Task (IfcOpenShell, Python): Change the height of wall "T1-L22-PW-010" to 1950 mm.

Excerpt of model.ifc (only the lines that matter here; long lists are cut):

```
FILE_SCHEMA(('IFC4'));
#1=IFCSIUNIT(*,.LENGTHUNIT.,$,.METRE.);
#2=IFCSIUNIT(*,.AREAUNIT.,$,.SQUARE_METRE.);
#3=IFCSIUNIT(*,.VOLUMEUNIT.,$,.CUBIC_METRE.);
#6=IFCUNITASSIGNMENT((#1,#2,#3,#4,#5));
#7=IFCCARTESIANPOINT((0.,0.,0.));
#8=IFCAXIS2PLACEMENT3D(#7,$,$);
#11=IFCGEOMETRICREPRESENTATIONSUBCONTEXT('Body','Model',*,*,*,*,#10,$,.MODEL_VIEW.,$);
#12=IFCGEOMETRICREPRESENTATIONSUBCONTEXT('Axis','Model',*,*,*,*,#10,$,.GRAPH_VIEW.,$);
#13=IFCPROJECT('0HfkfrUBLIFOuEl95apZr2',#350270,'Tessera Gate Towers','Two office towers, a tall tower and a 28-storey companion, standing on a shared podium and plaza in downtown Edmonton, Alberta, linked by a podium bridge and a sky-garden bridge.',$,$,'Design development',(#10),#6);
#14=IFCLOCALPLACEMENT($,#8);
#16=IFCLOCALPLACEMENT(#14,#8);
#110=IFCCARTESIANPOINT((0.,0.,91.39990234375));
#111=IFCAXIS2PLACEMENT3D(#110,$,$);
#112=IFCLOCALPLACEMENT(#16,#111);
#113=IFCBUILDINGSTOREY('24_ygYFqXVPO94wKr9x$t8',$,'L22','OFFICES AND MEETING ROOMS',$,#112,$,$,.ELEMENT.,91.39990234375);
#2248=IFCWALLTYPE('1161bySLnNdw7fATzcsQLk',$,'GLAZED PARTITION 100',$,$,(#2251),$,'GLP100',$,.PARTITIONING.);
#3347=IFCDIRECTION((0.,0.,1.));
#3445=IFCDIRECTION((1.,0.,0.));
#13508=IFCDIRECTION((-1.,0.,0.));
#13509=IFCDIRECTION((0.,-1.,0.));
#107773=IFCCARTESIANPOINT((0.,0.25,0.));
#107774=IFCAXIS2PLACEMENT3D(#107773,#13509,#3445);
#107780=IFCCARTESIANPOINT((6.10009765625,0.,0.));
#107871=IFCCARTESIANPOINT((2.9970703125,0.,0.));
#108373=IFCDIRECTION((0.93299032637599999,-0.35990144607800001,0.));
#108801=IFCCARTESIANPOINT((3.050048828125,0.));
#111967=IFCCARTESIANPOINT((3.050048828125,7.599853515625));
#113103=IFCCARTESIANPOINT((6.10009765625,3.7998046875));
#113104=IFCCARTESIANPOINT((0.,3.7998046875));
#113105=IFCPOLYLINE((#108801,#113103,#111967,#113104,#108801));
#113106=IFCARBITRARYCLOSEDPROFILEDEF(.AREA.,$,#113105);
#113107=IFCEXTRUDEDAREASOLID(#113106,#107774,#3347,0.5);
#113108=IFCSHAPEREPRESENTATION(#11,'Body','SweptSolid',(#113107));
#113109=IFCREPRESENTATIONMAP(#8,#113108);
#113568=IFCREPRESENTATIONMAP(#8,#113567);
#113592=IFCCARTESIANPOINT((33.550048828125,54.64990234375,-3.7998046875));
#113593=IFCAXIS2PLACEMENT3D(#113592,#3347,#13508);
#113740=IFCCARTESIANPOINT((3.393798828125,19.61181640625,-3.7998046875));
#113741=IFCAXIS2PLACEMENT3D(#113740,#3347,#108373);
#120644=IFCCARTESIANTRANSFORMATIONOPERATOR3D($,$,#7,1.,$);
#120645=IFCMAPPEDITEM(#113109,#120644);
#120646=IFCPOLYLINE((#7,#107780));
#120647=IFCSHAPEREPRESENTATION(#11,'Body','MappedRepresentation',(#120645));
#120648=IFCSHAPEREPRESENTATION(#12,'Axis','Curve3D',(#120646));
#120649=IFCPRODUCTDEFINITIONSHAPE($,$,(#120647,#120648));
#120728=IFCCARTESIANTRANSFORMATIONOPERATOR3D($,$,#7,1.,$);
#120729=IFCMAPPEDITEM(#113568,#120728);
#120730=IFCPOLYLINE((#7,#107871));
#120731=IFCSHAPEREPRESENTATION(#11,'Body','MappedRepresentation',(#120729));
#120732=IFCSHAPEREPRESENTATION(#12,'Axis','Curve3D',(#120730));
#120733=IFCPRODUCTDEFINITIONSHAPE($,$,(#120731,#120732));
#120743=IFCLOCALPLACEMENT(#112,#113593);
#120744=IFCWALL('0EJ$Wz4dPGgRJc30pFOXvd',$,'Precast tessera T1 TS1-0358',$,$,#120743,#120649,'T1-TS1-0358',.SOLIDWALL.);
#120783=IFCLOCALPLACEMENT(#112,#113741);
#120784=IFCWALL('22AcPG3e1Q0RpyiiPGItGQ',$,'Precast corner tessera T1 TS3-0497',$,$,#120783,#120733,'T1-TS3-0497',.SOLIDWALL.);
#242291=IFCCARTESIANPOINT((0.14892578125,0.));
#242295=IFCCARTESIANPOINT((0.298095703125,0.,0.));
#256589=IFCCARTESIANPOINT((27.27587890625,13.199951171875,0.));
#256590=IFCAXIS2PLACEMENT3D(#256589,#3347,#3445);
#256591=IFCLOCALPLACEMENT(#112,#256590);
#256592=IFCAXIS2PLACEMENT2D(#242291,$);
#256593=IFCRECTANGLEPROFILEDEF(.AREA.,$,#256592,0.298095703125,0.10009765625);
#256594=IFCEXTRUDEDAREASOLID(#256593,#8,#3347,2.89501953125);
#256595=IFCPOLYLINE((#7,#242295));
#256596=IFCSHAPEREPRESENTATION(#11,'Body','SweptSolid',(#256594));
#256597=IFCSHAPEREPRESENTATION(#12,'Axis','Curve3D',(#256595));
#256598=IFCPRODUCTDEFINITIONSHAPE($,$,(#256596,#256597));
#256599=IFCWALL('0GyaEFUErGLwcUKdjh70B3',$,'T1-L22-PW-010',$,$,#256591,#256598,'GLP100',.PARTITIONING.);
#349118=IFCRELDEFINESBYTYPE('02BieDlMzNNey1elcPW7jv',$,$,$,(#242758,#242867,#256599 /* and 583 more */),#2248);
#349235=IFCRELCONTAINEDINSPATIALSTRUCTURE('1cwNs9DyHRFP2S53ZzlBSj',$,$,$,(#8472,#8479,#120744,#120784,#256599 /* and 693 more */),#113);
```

```python
import ifcopenshell
import ifcopenshell.geom
import ifcopenshell.util.representation
import ifcopenshell.util.shape

model = ifcopenshell.open("model.ifc")
settings = ifcopenshell.geom.settings()


def volume(element):
    """Net volume in cubic metres, openings subtracted."""
    shape = ifcopenshell.geom.create_shape(settings, element)
    return ifcopenshell.util.shape.get_volume(shape.geometry)


wall = model.by_id(256599)
before = volume(wall)

body = ifcopenshell.util.representation.get_representation(wall, "Model", "Body")
solid = body.Items[0]
old_height = solid.Depth
solid.Depth = 1.95
after = volume(wall)

print(f"height {old_height:g} -> {solid.Depth:g}, volume {before:.3f} -> {after:.3f} m3")

model.write("model_edited.ifc")
```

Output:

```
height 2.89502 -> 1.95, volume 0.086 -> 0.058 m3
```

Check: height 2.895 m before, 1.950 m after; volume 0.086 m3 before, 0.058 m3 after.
